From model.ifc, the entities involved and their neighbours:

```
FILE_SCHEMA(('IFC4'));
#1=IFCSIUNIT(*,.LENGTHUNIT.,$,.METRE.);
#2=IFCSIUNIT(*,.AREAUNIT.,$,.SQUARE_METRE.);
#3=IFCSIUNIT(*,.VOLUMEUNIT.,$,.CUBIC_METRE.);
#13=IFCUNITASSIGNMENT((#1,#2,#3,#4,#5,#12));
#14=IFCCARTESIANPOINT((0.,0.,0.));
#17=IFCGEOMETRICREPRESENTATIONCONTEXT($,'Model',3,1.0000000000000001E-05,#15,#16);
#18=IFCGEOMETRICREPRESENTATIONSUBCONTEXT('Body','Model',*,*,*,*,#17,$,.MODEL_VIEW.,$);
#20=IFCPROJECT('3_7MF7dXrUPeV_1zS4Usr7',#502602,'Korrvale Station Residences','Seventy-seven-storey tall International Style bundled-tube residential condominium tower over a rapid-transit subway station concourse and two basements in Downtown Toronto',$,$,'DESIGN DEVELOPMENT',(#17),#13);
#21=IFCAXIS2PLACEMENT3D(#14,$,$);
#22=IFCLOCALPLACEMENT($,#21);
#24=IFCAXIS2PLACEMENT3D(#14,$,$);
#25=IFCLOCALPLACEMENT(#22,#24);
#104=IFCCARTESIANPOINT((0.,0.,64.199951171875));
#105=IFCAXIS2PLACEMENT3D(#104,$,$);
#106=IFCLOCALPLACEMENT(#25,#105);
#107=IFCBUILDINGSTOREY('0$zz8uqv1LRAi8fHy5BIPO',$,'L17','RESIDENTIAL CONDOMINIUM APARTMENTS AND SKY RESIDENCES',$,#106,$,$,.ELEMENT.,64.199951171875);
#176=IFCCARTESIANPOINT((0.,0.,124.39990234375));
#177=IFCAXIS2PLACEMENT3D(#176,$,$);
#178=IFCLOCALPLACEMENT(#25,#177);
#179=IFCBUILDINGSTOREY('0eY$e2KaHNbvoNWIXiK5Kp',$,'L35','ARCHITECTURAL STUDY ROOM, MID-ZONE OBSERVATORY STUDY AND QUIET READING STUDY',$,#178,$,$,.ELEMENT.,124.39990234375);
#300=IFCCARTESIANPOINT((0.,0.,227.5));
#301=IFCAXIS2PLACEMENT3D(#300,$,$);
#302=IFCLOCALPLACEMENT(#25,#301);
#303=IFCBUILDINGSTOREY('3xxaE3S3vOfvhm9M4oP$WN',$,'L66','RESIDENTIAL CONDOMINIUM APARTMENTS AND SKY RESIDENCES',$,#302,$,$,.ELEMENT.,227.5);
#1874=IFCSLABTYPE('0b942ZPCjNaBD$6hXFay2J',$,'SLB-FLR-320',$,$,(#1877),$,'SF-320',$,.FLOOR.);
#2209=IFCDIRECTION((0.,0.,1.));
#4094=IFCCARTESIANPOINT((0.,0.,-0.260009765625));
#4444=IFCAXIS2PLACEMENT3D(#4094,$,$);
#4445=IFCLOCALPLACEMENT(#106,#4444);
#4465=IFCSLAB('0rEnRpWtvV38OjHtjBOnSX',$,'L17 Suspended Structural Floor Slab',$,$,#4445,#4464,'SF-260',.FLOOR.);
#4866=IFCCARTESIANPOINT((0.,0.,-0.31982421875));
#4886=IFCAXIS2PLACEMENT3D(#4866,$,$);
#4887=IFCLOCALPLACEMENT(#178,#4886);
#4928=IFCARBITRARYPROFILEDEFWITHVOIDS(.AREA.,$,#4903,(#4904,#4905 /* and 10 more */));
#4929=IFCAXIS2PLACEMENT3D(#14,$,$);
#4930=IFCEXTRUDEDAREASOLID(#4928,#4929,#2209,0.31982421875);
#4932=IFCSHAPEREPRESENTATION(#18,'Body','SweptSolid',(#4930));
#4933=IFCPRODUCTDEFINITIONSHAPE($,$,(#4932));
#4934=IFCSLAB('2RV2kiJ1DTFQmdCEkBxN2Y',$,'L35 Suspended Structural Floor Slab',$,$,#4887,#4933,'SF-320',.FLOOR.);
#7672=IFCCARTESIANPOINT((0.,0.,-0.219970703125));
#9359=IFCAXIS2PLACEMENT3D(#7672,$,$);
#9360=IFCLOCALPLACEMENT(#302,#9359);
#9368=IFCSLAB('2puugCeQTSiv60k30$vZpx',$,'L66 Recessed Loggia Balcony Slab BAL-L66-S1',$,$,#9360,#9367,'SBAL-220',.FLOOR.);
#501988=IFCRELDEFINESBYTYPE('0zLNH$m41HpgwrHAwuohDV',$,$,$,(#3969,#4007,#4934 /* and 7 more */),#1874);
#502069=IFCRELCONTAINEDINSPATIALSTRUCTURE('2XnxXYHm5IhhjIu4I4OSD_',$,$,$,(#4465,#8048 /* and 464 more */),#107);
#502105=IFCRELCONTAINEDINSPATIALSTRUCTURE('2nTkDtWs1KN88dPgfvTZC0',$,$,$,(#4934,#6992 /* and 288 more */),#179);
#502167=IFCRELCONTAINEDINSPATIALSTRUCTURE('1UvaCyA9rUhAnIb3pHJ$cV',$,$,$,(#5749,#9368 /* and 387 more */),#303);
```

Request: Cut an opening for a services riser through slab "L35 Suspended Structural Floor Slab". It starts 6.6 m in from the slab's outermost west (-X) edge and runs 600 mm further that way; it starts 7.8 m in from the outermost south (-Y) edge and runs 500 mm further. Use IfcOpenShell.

```python
import numpy as np
import ifcopenshell
import ifcopenshell.api.feature
import ifcopenshell.api.geometry
import ifcopenshell.api.root
import ifcopenshell.geom
import ifcopenshell.util.placement
import ifcopenshell.util.representation
import ifcopenshell.util.shape
import ifcopenshell.util.unit

model = ifcopenshell.open("model.ifc")
unit_scale = ifcopenshell.util.unit.calculate_unit_scale(model)
settings = ifcopenshell.geom.settings()


def volume(element):
    """Net volume in cubic metres, openings subtracted."""
    shape = ifcopenshell.geom.create_shape(settings, element)
    return ifcopenshell.util.shape.get_volume(shape.geometry)


slab = model.by_id(4934)
before = volume(slab)

# Extent in the slab's own axes, in metres. The edges named are its -X and -Y sides.
slab_shape = ifcopenshell.geom.create_shape(settings, slab)
vertices = ifcopenshell.util.shape.get_vertices(slab_shape.geometry)
x_min, y_min, bottom = vertices.min(axis=0)
top = vertices[:, 2].max()

opening = ifcopenshell.api.root.create_entity(model, ifc_class="IfcOpeningElement", name="Services riser opening", predefined_type="OPENING")
context = ifcopenshell.util.representation.get_context(model, "Model", "Body", "MODEL_VIEW")
width, depth = 0.6, 0.5
outline = [(0.0, 0.0), (width, 0.0), (width, depth), (0.0, depth), (0.0, 0.0)]
# Overshoot both faces by 50 mm so the cut is clean.
shape = ifcopenshell.api.geometry.add_slab_representation(
    model, context=context, depth=top - bottom + 0.1, polyline=outline
)
ifcopenshell.api.geometry.assign_representation(model, product=opening, representation=shape)

matrix = ifcopenshell.util.placement.get_local_placement(slab.ObjectPlacement)
matrix[:, 3] = matrix @ np.append(np.array([x_min + 6.6, y_min + 7.8, bottom - 0.05]) / unit_scale, 1.0)
ifcopenshell.api.geometry.edit_object_placement(model, product=opening, matrix=matrix, is_si=False)
ifcopenshell.api.feature.add_feature(model, feature=opening, element=slab)

after = volume(slab)

print(f"slab volume {before:.3f} -> {after:.3f} m3")

model.write("model_edited.ifc")
```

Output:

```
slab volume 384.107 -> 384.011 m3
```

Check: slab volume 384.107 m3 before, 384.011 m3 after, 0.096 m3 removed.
